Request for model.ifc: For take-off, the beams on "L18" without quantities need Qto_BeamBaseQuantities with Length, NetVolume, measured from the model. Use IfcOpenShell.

First a look at what the model holds.

```python
import ifcopenshell
import ifcopenshell.util.element
import ifcopenshell.util.unit

model = ifcopenshell.open("model.ifc")
print(model.schema)
for unit_type in ("LENGTHUNIT", "AREAUNIT", "VOLUMEUNIT"):
    print(unit_type, ifcopenshell.util.unit.calculate_unit_scale(model, unit_type))
storey = next(s for s in model.by_type("IfcBuildingStorey") if s.Name == "L18")
beams = [e for e in ifcopenshell.util.element.get_decomposition(storey) if e.is_a("IfcBeam")]
for e in sorted(beams, key=lambda e: e.id()):
    print(e.id(), e.is_a(), e.Name, list(ifcopenshell.util.element.get_psets(e, qtos_only=True)), sep=" | ")
```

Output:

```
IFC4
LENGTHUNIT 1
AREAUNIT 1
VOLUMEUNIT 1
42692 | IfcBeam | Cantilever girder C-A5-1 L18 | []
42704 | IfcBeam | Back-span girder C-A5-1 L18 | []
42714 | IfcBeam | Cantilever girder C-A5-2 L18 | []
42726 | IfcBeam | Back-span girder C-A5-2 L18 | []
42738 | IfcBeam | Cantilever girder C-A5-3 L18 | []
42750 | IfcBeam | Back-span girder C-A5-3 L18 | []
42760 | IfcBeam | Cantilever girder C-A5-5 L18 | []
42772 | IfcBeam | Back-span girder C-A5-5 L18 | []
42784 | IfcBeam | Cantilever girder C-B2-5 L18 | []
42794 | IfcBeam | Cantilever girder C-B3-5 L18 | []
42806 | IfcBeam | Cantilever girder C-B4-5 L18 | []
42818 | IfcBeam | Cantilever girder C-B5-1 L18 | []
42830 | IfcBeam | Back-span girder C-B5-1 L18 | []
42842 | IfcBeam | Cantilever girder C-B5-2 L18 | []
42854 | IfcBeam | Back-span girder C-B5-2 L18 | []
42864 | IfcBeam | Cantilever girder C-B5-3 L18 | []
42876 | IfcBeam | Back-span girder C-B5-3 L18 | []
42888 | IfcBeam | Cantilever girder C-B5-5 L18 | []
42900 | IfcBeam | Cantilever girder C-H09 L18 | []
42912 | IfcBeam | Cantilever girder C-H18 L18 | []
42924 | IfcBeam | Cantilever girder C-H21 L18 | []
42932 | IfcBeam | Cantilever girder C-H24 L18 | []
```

```python
import ifcopenshell
import ifcopenshell.api.pset
import ifcopenshell.geom
import ifcopenshell.util.element
import ifcopenshell.util.shape
import ifcopenshell.util.unit

model = ifcopenshell.open("model.ifc")
unit_scale = ifcopenshell.util.unit.calculate_unit_scale(model)
volume_scale = ifcopenshell.util.unit.calculate_unit_scale(model, "VOLUMEUNIT")
settings = ifcopenshell.geom.settings()

storey = next(s for s in model.by_type("IfcBuildingStorey") if s.Name == "L18")
beams = [e for e in ifcopenshell.util.element.get_decomposition(storey) if e.is_a("IfcBeam")]

for e in sorted(beams, key=lambda e: e.id()):
    if ifcopenshell.util.element.get_psets(e, qtos_only=True, should_inherit=False):
        continue
    # Geometry comes back in metres, in the element's own axes.
    shape = ifcopenshell.geom.create_shape(settings, e)
    values = {
        "Length": ifcopenshell.util.shape.get_max_xyz(shape.geometry) / unit_scale,
        "NetVolume": ifcopenshell.util.shape.get_volume(shape.geometry) / volume_scale,
    }
    qto = ifcopenshell.api.pset.add_qto(model, product=e, name="Qto_BeamBaseQuantities")
    ifcopenshell.api.pset.edit_qto(model, qto=qto, properties=values)
    print(e.id(), {k: round(v, 3) for k, v in values.items()})

model.write("model_edited.ifc")
```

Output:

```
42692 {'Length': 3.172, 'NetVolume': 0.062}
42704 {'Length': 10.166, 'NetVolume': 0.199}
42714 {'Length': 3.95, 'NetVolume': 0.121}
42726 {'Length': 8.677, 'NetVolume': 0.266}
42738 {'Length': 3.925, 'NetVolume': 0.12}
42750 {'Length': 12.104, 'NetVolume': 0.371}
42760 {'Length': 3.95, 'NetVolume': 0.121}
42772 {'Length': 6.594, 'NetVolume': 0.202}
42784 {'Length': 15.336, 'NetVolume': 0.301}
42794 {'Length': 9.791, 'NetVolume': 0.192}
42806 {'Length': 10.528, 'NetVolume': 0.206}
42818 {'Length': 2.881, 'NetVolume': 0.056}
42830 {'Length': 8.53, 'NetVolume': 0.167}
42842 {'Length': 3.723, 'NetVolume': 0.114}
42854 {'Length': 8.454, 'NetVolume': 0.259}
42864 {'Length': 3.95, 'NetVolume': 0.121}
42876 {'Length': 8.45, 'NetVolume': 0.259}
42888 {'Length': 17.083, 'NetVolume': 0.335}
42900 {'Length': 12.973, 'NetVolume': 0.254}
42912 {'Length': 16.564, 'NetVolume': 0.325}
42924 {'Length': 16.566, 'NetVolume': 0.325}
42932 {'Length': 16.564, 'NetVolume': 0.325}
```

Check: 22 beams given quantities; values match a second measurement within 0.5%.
